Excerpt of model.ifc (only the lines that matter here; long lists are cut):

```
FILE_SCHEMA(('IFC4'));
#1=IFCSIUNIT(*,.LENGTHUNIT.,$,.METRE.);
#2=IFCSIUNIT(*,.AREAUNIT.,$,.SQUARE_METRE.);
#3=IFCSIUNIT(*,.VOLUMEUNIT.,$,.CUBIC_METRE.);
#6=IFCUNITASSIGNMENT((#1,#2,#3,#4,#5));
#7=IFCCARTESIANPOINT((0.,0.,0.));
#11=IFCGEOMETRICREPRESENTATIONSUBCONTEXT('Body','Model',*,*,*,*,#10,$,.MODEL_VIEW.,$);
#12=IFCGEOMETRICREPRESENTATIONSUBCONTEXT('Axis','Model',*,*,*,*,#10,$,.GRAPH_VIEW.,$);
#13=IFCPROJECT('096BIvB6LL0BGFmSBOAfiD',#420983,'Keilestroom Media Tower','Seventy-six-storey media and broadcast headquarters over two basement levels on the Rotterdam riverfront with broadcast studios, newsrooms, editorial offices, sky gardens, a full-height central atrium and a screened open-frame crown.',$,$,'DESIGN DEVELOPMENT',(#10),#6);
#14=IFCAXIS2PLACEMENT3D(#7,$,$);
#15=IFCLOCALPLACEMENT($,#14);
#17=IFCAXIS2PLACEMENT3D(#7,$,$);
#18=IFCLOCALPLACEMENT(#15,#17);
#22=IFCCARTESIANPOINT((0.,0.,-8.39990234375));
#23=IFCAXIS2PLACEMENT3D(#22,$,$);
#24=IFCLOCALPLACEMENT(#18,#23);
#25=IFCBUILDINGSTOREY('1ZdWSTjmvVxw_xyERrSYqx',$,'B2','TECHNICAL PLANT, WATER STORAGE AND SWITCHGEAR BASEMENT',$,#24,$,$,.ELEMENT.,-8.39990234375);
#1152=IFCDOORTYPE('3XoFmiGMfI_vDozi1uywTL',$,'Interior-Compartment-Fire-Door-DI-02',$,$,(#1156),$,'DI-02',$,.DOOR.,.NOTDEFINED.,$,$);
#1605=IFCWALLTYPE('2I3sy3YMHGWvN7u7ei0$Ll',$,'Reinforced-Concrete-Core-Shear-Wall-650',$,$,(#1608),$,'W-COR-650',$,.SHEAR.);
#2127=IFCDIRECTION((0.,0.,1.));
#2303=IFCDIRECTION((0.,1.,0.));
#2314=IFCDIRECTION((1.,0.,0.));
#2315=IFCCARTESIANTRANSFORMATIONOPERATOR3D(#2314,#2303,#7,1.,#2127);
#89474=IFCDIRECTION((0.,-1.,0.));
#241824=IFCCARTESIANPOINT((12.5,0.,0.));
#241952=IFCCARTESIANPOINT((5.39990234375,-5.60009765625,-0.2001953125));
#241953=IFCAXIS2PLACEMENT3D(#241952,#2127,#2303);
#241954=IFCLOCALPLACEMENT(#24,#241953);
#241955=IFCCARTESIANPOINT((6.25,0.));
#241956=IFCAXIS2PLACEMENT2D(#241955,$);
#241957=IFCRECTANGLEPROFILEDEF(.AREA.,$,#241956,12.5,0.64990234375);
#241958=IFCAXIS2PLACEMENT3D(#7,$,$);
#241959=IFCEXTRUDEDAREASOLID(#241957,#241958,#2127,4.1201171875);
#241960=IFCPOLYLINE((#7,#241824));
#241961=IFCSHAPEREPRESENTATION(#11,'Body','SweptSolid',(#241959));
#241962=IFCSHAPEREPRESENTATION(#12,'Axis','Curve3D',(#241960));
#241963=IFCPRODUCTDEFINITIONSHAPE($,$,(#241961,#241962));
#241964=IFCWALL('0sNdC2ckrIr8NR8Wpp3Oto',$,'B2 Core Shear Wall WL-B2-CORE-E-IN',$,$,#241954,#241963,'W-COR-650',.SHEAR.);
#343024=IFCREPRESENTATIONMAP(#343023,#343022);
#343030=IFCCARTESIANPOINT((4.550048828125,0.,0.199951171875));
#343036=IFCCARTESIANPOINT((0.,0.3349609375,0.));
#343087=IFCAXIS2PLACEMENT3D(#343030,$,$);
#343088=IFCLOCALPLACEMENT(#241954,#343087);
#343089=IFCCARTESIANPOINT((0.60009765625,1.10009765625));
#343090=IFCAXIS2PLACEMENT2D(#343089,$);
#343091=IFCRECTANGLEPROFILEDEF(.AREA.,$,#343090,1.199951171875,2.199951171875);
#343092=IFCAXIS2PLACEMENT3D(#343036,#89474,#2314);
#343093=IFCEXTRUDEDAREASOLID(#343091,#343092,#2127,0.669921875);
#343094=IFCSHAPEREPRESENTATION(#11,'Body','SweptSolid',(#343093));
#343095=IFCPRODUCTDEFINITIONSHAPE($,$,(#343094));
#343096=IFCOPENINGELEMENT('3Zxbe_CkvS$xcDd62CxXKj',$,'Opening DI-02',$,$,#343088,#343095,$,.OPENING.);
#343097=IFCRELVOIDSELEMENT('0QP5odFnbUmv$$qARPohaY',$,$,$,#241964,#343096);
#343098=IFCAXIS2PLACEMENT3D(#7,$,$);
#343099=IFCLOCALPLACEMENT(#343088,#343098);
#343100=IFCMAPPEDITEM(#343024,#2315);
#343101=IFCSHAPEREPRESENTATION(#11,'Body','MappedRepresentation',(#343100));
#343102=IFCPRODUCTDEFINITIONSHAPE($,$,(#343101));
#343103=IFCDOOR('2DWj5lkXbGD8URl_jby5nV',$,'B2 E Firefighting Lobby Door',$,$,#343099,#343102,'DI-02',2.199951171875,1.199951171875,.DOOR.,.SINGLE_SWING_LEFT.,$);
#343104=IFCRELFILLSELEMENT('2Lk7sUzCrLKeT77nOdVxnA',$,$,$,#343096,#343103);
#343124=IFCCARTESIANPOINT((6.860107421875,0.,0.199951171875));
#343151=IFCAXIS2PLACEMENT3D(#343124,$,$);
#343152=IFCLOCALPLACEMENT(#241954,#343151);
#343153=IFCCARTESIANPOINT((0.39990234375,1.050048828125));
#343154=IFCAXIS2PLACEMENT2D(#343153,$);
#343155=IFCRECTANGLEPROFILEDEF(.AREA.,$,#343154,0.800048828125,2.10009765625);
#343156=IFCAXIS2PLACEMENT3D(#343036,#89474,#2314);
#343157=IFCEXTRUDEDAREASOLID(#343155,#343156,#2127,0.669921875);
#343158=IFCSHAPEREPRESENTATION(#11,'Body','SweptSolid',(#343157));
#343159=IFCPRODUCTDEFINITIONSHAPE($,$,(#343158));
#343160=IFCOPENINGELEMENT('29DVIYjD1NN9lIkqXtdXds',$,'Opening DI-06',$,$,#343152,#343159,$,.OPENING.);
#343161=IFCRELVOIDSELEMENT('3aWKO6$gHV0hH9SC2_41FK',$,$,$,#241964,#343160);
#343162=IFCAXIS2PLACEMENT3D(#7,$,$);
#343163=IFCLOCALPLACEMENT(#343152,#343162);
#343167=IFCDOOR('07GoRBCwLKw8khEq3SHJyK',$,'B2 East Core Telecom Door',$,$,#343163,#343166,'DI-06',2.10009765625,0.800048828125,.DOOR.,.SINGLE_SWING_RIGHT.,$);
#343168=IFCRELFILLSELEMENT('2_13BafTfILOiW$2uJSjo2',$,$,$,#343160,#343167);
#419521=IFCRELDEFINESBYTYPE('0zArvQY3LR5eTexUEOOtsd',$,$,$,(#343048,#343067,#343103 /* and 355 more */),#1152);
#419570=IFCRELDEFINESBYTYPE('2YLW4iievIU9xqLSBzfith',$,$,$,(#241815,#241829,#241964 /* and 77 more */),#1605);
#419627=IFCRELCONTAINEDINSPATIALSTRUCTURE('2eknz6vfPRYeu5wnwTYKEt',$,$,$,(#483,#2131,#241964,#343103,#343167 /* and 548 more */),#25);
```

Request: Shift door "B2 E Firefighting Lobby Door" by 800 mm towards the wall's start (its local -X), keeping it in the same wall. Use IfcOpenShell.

```python
import ifcopenshell
import ifcopenshell.api.geometry
import ifcopenshell.util.placement

model = ifcopenshell.open("model.ifc")

door = model.by_guid("2DWj5lkXbGD8URl_jby5nV")
opening = door.FillsVoids[0].RelatingOpeningElement
wall = opening.VoidsElements[0].RelatingBuildingElement

wall_matrix = ifcopenshell.util.placement.get_local_placement(wall.ObjectPlacement)
shift = wall_matrix[:3, 0] * -0.8
before = ifcopenshell.util.placement.get_local_placement(door.ObjectPlacement)[:3, 3].copy()

# The door is placed relative to its opening, so it follows when the opening moves.
matrix = ifcopenshell.util.placement.get_local_placement(opening.ObjectPlacement)
matrix[:3, 3] += shift
ifcopenshell.api.geometry.edit_object_placement(
    model, product=opening, matrix=matrix, is_si=False, should_transform_children=True
)

after = ifcopenshell.util.placement.get_local_placement(door.ObjectPlacement)[:3, 3]
print("door moved by", (after - before).round(3) + 0.0)

model.write("model_v2.ifc")
```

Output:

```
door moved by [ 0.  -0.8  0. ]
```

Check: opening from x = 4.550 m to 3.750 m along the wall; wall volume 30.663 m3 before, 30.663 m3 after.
